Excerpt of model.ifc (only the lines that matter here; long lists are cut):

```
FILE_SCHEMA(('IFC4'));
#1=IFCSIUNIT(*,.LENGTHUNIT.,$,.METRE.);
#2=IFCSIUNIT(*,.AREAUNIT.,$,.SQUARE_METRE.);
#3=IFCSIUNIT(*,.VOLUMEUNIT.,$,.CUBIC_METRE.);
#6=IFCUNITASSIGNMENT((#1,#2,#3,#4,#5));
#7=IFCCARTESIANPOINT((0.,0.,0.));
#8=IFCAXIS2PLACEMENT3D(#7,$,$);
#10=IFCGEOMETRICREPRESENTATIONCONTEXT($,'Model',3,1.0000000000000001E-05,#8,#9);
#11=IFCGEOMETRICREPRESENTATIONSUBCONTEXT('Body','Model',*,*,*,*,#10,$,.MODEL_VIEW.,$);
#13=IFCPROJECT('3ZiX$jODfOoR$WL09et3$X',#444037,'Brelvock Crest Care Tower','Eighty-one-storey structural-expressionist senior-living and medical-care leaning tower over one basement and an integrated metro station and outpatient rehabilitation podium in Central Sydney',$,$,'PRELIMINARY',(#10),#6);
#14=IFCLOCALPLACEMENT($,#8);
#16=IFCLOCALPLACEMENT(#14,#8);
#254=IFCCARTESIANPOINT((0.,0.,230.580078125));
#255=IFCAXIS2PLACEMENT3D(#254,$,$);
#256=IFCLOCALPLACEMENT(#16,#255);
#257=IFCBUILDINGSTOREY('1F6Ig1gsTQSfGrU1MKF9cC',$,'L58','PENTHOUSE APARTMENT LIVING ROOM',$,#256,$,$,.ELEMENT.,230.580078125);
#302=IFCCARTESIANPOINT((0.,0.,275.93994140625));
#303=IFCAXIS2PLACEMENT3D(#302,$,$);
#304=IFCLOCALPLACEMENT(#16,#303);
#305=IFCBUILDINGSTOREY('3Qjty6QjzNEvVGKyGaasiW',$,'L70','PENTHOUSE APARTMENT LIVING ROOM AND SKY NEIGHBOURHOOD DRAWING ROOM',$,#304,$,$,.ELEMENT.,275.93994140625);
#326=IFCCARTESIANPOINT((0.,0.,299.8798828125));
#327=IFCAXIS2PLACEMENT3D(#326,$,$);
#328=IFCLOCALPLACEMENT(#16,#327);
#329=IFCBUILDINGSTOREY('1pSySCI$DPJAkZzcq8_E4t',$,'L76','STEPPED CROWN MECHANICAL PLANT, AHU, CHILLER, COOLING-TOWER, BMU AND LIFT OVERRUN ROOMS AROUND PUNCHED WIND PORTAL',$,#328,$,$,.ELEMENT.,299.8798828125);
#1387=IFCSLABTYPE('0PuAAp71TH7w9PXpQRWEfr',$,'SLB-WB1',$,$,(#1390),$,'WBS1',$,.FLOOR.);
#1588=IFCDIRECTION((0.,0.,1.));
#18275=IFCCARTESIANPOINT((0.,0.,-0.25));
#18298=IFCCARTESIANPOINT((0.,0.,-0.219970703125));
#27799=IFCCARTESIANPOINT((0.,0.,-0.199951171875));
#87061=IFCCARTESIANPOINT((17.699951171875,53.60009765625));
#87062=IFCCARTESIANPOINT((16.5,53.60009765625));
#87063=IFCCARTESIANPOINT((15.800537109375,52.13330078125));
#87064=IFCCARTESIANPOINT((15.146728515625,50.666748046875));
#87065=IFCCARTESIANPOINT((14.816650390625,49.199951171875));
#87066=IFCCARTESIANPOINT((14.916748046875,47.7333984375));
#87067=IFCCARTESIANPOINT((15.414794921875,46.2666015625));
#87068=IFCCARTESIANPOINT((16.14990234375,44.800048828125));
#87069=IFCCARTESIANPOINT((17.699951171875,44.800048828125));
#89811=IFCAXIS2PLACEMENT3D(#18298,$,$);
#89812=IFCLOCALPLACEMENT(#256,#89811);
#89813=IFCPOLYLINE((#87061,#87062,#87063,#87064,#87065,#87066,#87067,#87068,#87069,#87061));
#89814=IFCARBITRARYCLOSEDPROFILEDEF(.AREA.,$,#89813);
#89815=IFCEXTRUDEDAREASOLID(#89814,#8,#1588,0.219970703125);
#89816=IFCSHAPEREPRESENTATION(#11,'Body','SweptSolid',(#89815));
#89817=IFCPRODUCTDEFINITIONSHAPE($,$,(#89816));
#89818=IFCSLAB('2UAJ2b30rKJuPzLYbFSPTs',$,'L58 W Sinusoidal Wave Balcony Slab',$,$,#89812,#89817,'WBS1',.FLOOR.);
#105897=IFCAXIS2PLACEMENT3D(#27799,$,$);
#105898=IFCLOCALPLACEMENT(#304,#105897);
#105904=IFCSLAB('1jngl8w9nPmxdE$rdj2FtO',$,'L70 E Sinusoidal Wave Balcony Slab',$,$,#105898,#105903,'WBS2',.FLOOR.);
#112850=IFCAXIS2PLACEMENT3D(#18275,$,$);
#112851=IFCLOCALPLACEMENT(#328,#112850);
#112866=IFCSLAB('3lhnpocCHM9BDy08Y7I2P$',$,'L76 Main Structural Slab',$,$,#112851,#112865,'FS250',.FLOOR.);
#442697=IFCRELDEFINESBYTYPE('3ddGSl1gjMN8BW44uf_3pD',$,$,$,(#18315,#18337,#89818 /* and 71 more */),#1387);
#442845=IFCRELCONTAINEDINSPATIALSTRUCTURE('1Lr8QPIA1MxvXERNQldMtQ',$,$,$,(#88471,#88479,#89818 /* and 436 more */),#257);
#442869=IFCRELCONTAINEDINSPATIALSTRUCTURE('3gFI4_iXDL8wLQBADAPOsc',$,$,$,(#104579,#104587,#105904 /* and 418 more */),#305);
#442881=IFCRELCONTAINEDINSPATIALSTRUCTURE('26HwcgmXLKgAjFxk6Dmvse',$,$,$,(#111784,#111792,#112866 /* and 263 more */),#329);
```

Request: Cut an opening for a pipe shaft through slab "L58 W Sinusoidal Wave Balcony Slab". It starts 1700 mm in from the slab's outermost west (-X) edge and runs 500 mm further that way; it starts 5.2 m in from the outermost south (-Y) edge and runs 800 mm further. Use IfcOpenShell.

```python
import numpy as np
import ifcopenshell
import ifcopenshell.api.feature
import ifcopenshell.api.geometry
import ifcopenshell.api.root
import ifcopenshell.geom
import ifcopenshell.util.placement
import ifcopenshell.util.representation
import ifcopenshell.util.shape
import ifcopenshell.util.unit

model = ifcopenshell.open("model.ifc")
unit_scale = ifcopenshell.util.unit.calculate_unit_scale(model)
settings = ifcopenshell.geom.settings()


def volume(element):
    """Net volume in cubic metres, openings subtracted."""
    shape = ifcopenshell.geom.create_shape(settings, element)
    return ifcopenshell.util.shape.get_volume(shape.geometry)


slab = model.by_guid("2UAJ2b30rKJuPzLYbFSPTs")
before = volume(slab)

# Extent in the slab's own axes, in metres. The edges named are its -X and -Y sides.
slab_shape = ifcopenshell.geom.create_shape(settings, slab)
vertices = ifcopenshell.util.shape.get_vertices(slab_shape.geometry)
x_min, y_min, bottom = vertices.min(axis=0)
top = vertices[:, 2].max()

opening = ifcopenshell.api.root.create_entity(model, ifc_class="IfcOpeningElement", name="Pipe shaft opening", predefined_type="OPENING")
context = ifcopenshell.util.representation.get_context(model, "Model", "Body", "MODEL_VIEW")
width, depth = 0.5, 0.8
outline = [(0.0, 0.0), (width, 0.0), (width, depth), (0.0, depth), (0.0, 0.0)]
# Overshoot both faces by 50 mm so the cut is clean.
shape = ifcopenshell.api.geometry.add_slab_representation(
    model, context=context, depth=top - bottom + 0.1, polyline=outline
)
ifcopenshell.api.geometry.assign_representation(model, product=opening, representation=shape)

matrix = ifcopenshell.util.placement.get_local_placement(slab.ObjectPlacement)
matrix[:, 3] = matrix @ np.append(np.array([x_min + 1.7, y_min + 5.2, bottom - 0.05]) / unit_scale, 1.0)
ifcopenshell.api.geometry.edit_object_placement(model, product=opening, matrix=matrix, is_si=False)
ifcopenshell.api.feature.add_feature(model, feature=opening, element=slab)

after = volume(slab)

print(f"slab volume {before:.3f} -> {after:.3f} m3")

model.write("model_updated.ifc")
```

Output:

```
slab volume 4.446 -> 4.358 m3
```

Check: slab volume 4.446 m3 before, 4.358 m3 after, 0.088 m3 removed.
